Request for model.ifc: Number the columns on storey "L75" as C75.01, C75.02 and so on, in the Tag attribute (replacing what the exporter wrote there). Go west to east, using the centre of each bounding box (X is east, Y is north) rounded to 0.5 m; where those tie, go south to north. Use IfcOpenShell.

First a look at what the model holds.

```python
import ifcopenshell
import ifcopenshell.util.element
import ifcopenshell.util.placement

model = ifcopenshell.open("model.ifc")
print(model.schema)
storey = next(s for s in model.by_type("IfcBuildingStorey") if s.Name == "L75")
columns = [e for e in ifcopenshell.util.element.get_decomposition(storey) if e.is_a("IfcColumn")]
for e in sorted(columns, key=lambda e: e.id()):
    origin = ifcopenshell.util.placement.get_local_placement(e.ObjectPlacement)[:3, 3]
    print(e.id(), e.Tag, e.Name, origin.round(2) + 0.0, sep=" | ")
```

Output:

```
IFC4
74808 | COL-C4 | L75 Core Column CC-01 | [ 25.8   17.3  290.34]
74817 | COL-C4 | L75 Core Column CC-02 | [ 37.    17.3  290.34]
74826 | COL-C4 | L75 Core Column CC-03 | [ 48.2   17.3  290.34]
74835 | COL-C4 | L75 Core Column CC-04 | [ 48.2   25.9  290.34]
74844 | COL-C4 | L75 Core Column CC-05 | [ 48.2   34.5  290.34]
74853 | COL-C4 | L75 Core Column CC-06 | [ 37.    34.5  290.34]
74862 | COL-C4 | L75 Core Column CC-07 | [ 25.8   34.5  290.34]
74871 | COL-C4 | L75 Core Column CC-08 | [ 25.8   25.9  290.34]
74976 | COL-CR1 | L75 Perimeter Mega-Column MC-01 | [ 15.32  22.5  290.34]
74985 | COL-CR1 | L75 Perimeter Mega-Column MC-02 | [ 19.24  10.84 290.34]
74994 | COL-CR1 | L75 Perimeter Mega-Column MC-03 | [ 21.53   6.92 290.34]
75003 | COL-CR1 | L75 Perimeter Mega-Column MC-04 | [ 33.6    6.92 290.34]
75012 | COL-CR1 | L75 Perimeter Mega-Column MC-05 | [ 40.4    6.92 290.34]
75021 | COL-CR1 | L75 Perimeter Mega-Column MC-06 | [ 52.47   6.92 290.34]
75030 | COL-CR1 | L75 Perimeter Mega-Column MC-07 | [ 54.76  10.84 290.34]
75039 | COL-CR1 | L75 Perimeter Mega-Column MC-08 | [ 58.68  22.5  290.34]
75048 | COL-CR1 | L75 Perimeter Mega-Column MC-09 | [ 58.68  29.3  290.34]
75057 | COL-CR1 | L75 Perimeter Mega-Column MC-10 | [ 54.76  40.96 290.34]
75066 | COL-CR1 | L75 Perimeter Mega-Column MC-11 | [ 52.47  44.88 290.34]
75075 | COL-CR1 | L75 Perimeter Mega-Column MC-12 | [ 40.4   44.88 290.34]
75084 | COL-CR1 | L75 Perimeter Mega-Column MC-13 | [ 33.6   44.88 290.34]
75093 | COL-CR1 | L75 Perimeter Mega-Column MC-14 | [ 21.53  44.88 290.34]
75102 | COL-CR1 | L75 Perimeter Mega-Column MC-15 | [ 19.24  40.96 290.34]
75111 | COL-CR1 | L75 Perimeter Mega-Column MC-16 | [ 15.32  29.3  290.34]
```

```python
import ifcopenshell
import ifcopenshell.geom
import ifcopenshell.util.element
import ifcopenshell.util.shape

model = ifcopenshell.open("model.ifc")
settings = ifcopenshell.geom.settings()
settings.set("use-world-coords", True)


def centre(element):
    shape = ifcopenshell.geom.create_shape(settings, element)
    return ifcopenshell.util.shape.get_bbox_centroid(shape.geometry)


storey = next(s for s in model.by_type("IfcBuildingStorey") if s.Name == "L75")
columns = [e for e in ifcopenshell.util.element.get_decomposition(storey) if e.is_a("IfcColumn")]

# Insertion points can sit at a corner or the storey origin, so sort by the geometry (in metres).
centres = {e: centre(e) for e in columns}
columns.sort(key=lambda e: (round(centres[e][0] / 0.5), centres[e][1]))

for i, e in enumerate(columns, start=1):
    number = f"C75.{i:02d}"
    e.Tag = number
    print(e.id(), number)

model.write("model_rev.ifc")
```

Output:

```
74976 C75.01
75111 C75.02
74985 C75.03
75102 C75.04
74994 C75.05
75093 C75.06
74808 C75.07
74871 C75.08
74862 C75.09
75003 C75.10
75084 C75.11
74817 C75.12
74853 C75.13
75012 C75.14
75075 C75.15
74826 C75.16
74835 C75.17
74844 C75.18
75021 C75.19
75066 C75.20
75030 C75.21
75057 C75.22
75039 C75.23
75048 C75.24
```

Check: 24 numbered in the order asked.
